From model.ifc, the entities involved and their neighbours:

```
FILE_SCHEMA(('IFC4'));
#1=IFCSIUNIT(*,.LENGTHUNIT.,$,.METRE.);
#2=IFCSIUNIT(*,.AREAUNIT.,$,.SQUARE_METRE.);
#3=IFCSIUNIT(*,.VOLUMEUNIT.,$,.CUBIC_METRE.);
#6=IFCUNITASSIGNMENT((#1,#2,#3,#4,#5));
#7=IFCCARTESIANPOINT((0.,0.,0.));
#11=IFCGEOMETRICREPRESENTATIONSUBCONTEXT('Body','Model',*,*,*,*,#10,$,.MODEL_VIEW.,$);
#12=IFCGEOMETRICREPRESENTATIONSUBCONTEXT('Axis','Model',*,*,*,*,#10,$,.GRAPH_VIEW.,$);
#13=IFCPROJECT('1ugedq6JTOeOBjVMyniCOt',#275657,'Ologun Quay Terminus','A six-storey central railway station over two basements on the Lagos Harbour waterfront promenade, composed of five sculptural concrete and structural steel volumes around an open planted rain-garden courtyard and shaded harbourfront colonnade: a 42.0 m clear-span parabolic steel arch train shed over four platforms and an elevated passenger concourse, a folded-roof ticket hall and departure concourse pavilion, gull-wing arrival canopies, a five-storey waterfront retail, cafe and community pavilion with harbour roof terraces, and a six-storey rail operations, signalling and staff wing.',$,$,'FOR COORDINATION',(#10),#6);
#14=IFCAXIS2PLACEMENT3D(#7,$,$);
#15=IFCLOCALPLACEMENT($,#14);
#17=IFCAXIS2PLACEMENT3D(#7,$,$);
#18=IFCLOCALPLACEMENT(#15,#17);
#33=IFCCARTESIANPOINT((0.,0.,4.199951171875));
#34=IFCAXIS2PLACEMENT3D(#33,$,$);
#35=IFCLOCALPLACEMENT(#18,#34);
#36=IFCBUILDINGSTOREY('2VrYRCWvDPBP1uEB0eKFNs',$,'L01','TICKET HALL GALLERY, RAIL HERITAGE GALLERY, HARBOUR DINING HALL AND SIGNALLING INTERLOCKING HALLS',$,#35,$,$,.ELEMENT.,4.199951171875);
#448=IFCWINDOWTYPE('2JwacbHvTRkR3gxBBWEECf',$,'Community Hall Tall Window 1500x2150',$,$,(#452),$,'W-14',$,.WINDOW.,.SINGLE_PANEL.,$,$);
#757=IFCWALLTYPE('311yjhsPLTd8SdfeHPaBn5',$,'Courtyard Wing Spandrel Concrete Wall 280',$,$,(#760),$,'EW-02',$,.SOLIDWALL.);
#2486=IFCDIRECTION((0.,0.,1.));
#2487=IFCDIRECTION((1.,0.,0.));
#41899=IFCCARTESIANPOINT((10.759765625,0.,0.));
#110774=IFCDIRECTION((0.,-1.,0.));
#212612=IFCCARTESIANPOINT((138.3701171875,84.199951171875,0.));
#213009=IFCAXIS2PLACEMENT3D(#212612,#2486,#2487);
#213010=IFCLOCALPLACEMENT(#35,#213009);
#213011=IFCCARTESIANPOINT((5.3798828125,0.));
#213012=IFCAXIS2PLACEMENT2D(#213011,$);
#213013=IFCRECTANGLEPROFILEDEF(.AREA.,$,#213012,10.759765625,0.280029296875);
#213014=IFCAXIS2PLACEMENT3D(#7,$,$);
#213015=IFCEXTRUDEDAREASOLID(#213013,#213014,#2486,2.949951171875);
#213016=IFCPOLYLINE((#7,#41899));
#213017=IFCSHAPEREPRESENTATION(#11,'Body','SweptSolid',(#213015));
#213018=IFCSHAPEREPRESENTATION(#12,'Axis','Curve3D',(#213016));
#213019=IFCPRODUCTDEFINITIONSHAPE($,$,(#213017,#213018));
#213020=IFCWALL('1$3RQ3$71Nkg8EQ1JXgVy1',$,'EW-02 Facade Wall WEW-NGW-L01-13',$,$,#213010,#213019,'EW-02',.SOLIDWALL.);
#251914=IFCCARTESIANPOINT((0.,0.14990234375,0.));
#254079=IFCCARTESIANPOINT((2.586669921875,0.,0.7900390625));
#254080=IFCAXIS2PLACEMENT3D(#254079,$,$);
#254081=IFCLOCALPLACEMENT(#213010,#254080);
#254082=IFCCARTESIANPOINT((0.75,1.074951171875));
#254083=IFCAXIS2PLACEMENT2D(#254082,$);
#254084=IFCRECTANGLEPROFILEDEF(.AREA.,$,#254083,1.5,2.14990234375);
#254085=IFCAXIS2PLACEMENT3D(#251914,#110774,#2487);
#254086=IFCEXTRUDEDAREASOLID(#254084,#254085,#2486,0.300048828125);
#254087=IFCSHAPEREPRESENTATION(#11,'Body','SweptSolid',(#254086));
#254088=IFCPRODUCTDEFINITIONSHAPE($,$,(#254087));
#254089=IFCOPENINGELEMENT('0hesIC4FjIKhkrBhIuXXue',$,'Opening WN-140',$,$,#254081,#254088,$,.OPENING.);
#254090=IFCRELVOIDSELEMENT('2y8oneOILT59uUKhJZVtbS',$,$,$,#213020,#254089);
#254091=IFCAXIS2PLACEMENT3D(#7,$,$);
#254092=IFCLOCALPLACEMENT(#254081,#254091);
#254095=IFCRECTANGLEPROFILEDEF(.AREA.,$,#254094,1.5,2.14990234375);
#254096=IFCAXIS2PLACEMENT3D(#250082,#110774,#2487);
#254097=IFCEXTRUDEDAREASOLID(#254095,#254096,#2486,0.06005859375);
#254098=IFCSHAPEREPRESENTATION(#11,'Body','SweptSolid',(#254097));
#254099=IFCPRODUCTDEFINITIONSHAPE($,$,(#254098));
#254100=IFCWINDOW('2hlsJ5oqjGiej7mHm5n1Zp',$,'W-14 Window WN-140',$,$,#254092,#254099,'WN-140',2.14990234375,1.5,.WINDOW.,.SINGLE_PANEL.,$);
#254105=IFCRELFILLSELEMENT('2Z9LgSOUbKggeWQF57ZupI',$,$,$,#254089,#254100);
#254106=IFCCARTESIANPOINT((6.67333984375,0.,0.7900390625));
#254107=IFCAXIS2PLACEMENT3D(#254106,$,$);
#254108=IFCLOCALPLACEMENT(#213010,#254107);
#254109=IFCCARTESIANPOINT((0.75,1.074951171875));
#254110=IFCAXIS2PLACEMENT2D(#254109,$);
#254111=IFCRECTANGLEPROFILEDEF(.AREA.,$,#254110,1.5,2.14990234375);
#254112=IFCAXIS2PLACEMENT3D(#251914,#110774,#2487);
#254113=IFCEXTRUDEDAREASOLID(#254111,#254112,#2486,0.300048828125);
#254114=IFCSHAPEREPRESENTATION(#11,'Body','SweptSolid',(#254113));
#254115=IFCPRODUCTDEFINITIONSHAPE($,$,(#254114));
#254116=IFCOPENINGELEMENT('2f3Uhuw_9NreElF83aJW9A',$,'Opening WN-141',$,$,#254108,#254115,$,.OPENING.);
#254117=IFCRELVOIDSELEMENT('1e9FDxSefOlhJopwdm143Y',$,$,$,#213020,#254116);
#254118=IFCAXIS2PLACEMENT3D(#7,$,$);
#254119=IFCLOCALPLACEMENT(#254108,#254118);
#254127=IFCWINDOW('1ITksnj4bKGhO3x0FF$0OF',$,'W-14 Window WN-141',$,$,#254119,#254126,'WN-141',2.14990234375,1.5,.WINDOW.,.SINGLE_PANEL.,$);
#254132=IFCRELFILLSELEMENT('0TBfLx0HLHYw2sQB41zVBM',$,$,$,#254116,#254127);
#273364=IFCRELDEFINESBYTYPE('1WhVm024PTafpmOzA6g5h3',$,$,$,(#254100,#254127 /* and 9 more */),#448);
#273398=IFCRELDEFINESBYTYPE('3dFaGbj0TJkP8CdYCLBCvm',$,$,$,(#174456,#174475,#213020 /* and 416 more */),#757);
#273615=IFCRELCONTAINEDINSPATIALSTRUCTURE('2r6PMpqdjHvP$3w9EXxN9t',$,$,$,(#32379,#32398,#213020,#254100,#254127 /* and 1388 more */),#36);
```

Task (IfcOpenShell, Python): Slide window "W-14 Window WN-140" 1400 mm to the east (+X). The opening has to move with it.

```python
import ifcopenshell
import ifcopenshell.api.geometry
import ifcopenshell.util.placement
import ifcopenshell.util.unit

model = ifcopenshell.open("model.ifc")
unit_scale = ifcopenshell.util.unit.calculate_unit_scale(model)

window = model.by_guid("2hlsJ5oqjGiej7mHm5n1Zp")
opening = window.FillsVoids[0].RelatingOpeningElement
wall = opening.VoidsElements[0].RelatingBuildingElement

wall_matrix = ifcopenshell.util.placement.get_local_placement(wall.ObjectPlacement)
shift = wall_matrix[:3, 0] * 1.4 / unit_scale
before = ifcopenshell.util.placement.get_local_placement(window.ObjectPlacement)[:3, 3].copy()

# The window is placed relative to its opening, so it follows when the opening moves.
matrix = ifcopenshell.util.placement.get_local_placement(opening.ObjectPlacement)
matrix[:3, 3] += shift
ifcopenshell.api.geometry.edit_object_placement(
    model, product=opening, matrix=matrix, is_si=False, should_transform_children=True
)

after = ifcopenshell.util.placement.get_local_placement(window.ObjectPlacement)[:3, 3]
print("window moved by", (after - before).round(3) + 0.0)

model.write("model_rev.ifc")
```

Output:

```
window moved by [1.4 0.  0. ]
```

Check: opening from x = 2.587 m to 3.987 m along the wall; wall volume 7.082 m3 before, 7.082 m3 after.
